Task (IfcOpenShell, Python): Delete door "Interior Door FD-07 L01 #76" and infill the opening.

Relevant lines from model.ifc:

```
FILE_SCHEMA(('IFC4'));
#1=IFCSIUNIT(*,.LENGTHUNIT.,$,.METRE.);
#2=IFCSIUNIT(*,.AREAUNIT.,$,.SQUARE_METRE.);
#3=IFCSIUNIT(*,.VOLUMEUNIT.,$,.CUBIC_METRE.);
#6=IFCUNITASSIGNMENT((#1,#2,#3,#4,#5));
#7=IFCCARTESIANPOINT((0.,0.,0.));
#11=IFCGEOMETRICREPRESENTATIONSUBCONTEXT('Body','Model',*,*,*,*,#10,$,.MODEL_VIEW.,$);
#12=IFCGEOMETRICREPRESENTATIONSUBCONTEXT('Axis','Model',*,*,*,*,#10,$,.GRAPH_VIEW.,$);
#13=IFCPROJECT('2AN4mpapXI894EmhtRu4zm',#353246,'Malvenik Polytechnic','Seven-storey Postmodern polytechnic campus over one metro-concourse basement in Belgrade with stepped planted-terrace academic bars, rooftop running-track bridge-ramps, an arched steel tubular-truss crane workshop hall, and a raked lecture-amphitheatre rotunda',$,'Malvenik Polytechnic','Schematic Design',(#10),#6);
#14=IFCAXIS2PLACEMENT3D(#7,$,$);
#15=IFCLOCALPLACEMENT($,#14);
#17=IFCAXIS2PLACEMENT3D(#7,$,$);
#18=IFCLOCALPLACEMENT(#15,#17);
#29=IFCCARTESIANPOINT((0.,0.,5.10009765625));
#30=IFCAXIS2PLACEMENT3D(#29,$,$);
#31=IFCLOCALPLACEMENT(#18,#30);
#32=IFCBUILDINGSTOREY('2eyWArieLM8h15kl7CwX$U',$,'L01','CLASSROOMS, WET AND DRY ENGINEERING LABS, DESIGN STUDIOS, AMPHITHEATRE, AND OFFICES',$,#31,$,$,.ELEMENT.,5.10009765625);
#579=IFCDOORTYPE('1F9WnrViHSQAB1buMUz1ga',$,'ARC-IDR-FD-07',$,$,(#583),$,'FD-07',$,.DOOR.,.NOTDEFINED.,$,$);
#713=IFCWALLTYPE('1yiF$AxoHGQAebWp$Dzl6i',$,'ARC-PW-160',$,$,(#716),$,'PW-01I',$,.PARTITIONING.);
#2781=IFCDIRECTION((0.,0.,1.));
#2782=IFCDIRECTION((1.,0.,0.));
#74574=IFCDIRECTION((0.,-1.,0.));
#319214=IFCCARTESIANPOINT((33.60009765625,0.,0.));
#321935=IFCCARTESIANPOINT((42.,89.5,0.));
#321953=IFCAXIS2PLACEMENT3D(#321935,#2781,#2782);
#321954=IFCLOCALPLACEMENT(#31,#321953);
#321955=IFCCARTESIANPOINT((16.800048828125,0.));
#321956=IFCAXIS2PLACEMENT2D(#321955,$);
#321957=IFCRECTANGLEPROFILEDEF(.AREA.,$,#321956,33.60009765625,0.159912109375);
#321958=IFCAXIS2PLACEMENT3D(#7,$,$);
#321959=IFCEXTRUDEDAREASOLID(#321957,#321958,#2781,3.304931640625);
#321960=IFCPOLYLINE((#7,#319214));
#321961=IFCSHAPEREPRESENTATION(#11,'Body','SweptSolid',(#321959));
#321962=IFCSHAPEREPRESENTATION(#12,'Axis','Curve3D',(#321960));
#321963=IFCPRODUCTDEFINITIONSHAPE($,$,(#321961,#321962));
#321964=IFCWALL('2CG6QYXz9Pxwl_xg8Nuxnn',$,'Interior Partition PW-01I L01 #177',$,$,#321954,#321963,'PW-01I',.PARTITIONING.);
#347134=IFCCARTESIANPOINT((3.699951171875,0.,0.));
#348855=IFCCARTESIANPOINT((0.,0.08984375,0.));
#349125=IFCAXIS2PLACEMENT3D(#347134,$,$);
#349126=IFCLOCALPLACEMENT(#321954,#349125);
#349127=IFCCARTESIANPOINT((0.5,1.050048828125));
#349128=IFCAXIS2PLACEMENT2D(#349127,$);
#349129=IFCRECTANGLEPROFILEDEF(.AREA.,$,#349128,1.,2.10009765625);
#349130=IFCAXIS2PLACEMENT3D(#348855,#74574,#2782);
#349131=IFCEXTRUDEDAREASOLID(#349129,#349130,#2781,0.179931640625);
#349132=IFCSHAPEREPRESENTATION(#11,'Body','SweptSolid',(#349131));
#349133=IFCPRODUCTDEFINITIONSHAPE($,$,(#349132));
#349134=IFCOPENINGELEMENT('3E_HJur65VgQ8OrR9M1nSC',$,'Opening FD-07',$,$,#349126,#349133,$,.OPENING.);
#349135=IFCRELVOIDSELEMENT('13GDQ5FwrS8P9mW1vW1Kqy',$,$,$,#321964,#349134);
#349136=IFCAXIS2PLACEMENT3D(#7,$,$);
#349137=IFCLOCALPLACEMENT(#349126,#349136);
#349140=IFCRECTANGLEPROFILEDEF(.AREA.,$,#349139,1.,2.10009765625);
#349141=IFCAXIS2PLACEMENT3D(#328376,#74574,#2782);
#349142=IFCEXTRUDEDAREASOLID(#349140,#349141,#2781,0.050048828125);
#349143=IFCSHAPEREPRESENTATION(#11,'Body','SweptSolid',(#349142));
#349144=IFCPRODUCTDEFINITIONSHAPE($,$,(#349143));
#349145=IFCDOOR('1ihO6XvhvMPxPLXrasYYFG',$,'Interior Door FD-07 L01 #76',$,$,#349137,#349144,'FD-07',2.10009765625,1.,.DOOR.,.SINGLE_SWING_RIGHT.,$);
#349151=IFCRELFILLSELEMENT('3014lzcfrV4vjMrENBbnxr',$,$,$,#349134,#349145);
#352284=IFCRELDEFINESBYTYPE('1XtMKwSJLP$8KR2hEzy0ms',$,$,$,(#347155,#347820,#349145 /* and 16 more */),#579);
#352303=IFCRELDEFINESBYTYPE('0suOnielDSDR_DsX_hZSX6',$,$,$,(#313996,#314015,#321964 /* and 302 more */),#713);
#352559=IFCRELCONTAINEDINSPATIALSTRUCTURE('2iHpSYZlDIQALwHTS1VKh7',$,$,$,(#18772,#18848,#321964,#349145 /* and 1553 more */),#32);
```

```python
import ifcopenshell
import ifcopenshell.api.feature
import ifcopenshell.api.root
import ifcopenshell.geom
import ifcopenshell.util.shape

model = ifcopenshell.open("model.ifc")
settings = ifcopenshell.geom.settings()


def volume(element):
    """Net volume in cubic metres, openings subtracted."""
    shape = ifcopenshell.geom.create_shape(settings, element)
    return ifcopenshell.util.shape.get_volume(shape.geometry)


door = model.by_guid("1ihO6XvhvMPxPLXrasYYFG")
opening = door.FillsVoids[0].RelatingOpeningElement
wall = opening.VoidsElements[0].RelatingBuildingElement
before = volume(wall)

ifcopenshell.api.root.remove_product(model, product=door)
ifcopenshell.api.feature.remove_feature(model, feature=opening)

after = volume(wall)

print(f"wall volume {before:.3f} -> {after:.3f} m3")

model.write("model_rev.ifc")
```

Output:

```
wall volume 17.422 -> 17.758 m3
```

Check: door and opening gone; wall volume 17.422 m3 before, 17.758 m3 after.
